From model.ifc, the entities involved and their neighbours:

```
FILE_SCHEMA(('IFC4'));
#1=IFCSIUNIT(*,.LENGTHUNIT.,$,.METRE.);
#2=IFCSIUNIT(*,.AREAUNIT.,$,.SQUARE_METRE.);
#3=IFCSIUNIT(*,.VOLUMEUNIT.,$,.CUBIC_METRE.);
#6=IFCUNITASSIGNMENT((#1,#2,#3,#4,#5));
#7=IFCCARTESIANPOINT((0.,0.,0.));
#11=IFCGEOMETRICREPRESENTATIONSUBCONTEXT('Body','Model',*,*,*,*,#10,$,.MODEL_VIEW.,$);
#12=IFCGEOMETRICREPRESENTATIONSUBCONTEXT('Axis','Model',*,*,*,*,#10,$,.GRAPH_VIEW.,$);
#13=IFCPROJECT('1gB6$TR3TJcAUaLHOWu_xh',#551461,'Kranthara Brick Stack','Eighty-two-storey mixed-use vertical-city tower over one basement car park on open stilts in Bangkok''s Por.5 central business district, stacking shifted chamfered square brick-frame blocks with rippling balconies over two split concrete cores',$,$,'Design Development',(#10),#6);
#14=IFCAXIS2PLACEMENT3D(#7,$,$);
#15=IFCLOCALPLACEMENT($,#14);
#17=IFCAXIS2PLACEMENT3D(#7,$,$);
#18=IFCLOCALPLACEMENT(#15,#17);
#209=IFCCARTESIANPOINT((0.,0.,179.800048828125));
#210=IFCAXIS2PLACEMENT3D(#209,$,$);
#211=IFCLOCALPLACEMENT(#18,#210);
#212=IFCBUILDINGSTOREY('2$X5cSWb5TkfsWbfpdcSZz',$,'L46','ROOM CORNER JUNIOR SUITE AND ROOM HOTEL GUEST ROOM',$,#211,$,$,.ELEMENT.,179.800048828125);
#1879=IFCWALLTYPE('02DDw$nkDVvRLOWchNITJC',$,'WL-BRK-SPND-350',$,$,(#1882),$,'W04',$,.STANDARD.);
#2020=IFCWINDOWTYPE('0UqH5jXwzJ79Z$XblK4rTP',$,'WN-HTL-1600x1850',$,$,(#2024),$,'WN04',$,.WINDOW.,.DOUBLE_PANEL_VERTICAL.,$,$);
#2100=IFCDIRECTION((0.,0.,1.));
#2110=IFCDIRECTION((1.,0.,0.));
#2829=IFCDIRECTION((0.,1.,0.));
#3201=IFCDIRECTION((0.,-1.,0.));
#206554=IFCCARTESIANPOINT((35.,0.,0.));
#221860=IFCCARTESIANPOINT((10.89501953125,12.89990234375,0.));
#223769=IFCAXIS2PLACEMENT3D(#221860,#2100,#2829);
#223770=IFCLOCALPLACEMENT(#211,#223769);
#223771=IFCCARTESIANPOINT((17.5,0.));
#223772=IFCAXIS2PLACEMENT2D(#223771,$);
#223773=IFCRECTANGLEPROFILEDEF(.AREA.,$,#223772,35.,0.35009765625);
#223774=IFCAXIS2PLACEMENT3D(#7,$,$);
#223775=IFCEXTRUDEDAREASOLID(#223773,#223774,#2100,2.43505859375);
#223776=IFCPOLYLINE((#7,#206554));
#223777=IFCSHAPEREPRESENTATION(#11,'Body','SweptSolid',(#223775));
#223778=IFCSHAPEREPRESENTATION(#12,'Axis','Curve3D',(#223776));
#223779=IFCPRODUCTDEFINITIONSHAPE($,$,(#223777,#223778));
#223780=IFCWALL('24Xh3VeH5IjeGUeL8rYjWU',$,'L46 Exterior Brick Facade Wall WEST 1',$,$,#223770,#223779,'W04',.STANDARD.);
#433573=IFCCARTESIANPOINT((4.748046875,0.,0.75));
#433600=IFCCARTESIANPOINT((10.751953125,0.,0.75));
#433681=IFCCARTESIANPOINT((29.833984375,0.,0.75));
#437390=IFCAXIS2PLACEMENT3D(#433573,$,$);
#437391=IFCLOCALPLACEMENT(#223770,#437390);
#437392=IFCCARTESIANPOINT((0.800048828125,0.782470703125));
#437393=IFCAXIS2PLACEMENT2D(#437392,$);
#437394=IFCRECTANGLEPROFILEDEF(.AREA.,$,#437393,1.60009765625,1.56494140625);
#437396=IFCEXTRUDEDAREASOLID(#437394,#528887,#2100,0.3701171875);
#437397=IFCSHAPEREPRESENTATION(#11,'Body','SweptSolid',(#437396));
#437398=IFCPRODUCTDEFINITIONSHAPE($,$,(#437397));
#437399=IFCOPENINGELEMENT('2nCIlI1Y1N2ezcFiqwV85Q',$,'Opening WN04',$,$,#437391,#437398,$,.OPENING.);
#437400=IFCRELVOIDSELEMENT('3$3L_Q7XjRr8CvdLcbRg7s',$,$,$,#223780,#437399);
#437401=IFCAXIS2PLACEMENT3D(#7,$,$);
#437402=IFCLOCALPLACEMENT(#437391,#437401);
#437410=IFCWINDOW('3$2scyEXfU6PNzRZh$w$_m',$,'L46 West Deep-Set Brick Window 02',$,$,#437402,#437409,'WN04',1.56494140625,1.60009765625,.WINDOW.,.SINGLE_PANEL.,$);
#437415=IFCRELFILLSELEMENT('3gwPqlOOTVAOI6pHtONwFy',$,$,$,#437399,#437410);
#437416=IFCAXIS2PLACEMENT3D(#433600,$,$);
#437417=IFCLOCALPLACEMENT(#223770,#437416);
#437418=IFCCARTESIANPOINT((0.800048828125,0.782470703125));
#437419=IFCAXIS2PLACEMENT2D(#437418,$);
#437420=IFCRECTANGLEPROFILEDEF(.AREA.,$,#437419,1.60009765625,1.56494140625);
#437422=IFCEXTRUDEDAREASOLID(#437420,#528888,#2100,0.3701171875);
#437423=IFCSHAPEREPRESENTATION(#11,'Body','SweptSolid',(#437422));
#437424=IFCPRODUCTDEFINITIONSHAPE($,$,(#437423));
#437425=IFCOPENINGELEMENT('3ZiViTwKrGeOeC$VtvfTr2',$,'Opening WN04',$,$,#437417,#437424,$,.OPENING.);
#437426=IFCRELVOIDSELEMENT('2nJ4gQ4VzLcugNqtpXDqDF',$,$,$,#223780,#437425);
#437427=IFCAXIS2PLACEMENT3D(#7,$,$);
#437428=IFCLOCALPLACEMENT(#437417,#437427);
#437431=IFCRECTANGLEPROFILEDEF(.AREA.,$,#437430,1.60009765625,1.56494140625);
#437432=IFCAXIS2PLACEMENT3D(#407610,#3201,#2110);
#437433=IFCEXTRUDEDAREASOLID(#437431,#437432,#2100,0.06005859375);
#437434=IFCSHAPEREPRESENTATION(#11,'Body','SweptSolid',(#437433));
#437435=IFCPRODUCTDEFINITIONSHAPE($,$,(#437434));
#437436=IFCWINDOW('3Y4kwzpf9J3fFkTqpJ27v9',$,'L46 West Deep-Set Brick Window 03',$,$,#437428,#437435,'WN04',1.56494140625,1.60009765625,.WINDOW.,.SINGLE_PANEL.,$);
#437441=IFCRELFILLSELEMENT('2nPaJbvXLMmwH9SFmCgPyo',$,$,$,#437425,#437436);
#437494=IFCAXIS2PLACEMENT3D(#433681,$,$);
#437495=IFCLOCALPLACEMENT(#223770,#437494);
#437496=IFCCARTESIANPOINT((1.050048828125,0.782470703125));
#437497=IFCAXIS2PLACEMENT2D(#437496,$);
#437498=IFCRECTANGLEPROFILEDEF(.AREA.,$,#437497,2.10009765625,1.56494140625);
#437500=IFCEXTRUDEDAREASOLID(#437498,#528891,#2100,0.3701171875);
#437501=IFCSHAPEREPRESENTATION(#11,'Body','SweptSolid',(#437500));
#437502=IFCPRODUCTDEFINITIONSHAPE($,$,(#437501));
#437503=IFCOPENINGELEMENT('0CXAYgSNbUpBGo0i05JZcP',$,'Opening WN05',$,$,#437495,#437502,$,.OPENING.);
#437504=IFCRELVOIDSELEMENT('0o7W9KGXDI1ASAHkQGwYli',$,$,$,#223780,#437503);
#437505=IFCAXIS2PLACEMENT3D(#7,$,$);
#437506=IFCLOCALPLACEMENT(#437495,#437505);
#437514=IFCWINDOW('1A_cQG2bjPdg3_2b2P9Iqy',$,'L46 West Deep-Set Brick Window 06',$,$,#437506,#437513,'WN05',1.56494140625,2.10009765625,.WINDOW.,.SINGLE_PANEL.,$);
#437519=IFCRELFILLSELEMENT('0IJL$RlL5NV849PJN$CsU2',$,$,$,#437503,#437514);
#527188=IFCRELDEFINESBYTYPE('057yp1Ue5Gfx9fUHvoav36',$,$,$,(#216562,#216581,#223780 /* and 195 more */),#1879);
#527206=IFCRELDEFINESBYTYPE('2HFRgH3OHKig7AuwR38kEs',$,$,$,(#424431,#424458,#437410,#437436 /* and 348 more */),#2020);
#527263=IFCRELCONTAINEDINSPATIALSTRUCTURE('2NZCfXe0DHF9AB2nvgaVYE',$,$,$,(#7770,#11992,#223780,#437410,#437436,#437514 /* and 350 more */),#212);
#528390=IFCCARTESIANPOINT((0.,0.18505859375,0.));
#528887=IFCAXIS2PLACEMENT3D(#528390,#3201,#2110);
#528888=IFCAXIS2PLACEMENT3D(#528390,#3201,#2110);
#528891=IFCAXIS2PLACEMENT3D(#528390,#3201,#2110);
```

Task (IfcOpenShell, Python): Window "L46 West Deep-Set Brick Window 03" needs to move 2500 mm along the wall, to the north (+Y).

```python
import ifcopenshell
import ifcopenshell.api.geometry
import ifcopenshell.util.placement

model = ifcopenshell.open("model.ifc")

window = model.by_guid("3Y4kwzpf9J3fFkTqpJ27v9")
opening = window.FillsVoids[0].RelatingOpeningElement
wall = opening.VoidsElements[0].RelatingBuildingElement

wall_matrix = ifcopenshell.util.placement.get_local_placement(wall.ObjectPlacement)
shift = wall_matrix[:3, 0] * 2.5
before = ifcopenshell.util.placement.get_local_placement(window.ObjectPlacement)[:3, 3].copy()

# The window is placed relative to its opening, so it follows when the opening moves.
matrix = ifcopenshell.util.placement.get_local_placement(opening.ObjectPlacement)
matrix[:3, 3] += shift
ifcopenshell.api.geometry.edit_object_placement(
    model, product=opening, matrix=matrix, is_si=False, should_transform_children=True
)

after = ifcopenshell.util.placement.get_local_placement(window.ObjectPlacement)[:3, 3]
print("window moved by", (after - before).round(3) + 0.0)

model.write("model_updated.ifc")
```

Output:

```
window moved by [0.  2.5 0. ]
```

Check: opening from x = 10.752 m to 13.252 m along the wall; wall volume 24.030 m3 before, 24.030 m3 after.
